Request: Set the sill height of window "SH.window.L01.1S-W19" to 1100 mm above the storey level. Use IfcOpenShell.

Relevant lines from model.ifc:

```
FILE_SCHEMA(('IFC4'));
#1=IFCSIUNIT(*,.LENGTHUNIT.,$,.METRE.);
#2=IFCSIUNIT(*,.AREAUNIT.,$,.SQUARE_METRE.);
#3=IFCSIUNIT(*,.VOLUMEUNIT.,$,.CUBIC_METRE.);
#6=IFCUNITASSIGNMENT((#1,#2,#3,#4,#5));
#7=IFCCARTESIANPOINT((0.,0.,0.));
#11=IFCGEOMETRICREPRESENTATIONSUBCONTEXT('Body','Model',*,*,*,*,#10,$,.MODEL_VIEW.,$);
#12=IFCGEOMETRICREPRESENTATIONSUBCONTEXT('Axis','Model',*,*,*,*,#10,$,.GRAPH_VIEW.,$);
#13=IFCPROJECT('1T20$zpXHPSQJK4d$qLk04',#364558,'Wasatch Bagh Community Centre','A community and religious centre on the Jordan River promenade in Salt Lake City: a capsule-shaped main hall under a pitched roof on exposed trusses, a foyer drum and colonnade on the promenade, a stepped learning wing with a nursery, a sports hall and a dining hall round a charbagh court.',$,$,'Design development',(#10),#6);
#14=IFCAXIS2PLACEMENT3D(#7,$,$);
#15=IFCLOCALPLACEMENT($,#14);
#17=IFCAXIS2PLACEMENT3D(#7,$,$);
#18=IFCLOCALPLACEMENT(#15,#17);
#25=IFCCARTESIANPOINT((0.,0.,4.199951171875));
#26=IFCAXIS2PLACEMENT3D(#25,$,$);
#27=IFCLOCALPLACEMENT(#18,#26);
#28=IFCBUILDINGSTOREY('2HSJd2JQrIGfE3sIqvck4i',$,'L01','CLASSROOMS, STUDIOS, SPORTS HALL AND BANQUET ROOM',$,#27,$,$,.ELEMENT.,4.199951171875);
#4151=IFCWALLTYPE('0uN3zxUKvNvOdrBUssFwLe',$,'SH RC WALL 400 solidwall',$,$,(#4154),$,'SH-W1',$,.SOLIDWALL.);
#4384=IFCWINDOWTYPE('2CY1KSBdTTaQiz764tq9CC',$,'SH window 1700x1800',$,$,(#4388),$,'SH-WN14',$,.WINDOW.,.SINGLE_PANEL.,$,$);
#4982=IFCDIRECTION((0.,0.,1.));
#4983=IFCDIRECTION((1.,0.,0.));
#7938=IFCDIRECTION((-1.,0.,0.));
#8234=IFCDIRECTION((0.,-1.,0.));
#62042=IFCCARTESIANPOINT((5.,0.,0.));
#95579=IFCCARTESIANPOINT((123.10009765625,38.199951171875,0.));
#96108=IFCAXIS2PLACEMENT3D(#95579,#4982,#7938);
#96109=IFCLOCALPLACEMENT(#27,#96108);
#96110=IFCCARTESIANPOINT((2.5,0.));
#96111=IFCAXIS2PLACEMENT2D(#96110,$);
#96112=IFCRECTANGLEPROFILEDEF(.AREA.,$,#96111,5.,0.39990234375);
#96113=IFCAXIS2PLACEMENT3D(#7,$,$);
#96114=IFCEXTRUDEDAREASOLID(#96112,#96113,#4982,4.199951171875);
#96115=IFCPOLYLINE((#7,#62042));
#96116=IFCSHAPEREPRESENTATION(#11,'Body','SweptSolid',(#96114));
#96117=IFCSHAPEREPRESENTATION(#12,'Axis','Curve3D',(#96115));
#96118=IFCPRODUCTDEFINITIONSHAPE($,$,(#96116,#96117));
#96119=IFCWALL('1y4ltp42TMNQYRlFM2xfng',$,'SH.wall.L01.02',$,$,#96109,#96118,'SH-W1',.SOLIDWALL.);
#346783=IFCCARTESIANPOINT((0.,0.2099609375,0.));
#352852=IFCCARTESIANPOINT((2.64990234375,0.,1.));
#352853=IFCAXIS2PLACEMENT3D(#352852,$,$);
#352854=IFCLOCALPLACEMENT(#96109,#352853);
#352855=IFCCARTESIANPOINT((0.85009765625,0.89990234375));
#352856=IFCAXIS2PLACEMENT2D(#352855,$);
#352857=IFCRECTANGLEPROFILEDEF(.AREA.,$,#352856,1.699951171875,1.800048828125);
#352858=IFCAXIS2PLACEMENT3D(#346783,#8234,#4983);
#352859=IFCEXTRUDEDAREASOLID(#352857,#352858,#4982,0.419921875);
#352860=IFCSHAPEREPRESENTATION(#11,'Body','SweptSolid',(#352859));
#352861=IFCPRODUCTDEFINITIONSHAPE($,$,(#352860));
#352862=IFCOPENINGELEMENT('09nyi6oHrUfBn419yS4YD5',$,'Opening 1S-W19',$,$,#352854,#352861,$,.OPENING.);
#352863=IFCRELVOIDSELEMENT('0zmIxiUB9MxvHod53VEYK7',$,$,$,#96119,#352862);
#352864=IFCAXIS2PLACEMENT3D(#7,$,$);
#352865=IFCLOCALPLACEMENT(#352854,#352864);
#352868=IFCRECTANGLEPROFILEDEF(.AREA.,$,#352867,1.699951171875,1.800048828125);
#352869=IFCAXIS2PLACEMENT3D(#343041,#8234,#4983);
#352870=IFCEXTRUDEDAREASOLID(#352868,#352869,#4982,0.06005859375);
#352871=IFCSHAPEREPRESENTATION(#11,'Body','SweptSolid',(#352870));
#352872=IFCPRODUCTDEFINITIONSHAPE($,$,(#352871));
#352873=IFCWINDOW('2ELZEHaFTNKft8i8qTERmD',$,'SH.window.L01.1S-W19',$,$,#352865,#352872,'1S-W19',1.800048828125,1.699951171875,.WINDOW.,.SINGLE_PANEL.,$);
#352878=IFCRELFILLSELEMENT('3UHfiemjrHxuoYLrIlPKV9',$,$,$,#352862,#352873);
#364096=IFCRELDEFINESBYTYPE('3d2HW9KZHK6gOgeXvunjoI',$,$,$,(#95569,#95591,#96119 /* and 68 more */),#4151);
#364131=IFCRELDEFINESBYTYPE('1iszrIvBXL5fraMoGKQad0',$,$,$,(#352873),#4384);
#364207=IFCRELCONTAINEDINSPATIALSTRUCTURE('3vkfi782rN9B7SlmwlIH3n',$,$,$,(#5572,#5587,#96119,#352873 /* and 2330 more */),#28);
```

```python
import numpy as np
import ifcopenshell
import ifcopenshell.api.geometry
import ifcopenshell.geom
import ifcopenshell.util.element
import ifcopenshell.util.placement
import ifcopenshell.util.shape
import ifcopenshell.util.unit

model = ifcopenshell.open("model.ifc")
unit_scale = ifcopenshell.util.unit.calculate_unit_scale(model)

window = model.by_guid("2ELZEHaFTNKft8i8qTERmD")
opening = window.FillsVoids[0].RelatingOpeningElement
storey = ifcopenshell.util.element.get_container(window, ifc_class="IfcBuildingStorey")
level = ifcopenshell.util.placement.get_local_placement(storey.ObjectPlacement)[2, 3]

# The opening's origin need not be at the sill, so measure its lowest point.
shape = ifcopenshell.geom.create_shape(ifcopenshell.geom.settings(), opening)
bottom = ifcopenshell.util.shape.get_shape_bottom_elevation(shape, shape.geometry) / unit_scale
dz = level + 1.1 - bottom

shift = np.array([0.0, 0.0, dz])
# The window is placed relative to its opening, so it follows when the opening moves.
matrix = ifcopenshell.util.placement.get_local_placement(opening.ObjectPlacement)
matrix[:3, 3] += shift
ifcopenshell.api.geometry.edit_object_placement(
    model, product=opening, matrix=matrix, is_si=False, should_transform_children=True
)

print(f"moved by {dz * unit_scale:+.3f} m")

model.write("model_updated.ifc")
```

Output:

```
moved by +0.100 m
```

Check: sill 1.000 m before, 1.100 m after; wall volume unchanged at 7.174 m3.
